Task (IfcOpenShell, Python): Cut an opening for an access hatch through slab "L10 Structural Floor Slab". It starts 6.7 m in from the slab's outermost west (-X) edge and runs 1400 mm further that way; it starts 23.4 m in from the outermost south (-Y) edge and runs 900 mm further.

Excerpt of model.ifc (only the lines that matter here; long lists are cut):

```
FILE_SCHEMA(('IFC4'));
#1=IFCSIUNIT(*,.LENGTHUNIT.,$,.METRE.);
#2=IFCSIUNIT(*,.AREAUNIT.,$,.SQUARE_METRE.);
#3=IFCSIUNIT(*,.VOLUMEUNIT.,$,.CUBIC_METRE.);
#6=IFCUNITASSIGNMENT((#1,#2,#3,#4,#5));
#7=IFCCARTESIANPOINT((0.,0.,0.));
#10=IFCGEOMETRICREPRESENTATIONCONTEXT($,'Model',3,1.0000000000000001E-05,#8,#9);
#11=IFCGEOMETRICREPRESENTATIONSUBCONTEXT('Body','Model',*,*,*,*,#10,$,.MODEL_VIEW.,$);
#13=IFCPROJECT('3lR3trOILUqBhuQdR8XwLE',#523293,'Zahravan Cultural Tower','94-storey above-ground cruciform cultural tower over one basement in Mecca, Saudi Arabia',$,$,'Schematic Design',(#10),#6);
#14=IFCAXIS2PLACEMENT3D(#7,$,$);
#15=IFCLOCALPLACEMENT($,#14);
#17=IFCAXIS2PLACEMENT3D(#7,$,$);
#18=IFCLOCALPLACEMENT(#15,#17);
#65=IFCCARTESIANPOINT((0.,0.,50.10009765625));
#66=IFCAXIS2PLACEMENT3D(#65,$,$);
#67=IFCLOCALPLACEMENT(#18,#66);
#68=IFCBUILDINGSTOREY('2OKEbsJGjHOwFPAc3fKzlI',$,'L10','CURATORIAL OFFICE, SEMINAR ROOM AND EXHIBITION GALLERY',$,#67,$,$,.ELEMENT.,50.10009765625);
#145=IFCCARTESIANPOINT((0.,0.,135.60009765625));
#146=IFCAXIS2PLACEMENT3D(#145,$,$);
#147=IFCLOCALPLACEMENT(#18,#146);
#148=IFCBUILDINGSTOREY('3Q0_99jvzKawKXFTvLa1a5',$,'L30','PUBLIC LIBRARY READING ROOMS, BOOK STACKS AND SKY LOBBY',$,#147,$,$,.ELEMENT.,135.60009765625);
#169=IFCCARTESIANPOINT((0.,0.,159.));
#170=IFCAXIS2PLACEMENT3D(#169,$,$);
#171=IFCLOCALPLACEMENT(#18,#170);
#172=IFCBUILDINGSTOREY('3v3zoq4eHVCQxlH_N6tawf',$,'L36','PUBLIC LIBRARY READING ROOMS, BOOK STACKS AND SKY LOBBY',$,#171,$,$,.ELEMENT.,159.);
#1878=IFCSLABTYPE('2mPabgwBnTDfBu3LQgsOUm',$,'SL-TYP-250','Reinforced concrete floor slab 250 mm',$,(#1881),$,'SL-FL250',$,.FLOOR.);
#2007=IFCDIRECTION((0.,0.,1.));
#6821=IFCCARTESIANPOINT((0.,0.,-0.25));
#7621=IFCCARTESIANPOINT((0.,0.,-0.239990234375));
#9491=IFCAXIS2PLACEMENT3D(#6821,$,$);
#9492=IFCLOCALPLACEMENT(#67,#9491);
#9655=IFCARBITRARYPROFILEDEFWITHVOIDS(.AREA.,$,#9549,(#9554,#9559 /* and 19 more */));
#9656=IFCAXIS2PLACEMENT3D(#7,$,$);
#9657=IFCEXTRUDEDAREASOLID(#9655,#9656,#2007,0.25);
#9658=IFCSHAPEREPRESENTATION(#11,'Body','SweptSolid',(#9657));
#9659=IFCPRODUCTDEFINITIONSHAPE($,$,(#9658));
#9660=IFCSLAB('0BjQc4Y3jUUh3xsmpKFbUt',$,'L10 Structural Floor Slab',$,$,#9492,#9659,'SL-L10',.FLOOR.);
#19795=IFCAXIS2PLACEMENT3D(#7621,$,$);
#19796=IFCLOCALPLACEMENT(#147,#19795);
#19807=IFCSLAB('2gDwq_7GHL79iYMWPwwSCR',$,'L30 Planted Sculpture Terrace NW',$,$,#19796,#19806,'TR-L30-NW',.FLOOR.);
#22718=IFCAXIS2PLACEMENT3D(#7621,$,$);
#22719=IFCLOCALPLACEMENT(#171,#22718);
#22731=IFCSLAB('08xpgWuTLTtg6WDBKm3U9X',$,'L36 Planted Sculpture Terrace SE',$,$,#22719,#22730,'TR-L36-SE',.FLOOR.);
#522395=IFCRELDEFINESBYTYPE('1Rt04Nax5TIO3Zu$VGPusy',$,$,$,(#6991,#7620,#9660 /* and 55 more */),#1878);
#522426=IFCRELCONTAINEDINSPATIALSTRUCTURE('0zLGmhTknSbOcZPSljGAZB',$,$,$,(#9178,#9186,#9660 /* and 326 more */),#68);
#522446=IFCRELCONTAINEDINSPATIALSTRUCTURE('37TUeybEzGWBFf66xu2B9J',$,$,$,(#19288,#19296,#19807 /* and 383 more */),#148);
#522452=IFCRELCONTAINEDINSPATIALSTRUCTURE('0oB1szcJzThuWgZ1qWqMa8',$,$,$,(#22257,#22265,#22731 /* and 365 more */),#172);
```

```python
import numpy as np
import ifcopenshell
import ifcopenshell.api.feature
import ifcopenshell.api.geometry
import ifcopenshell.api.root
import ifcopenshell.geom
import ifcopenshell.util.placement
import ifcopenshell.util.representation
import ifcopenshell.util.shape
import ifcopenshell.util.unit

model = ifcopenshell.open("model.ifc")
unit_scale = ifcopenshell.util.unit.calculate_unit_scale(model)
settings = ifcopenshell.geom.settings()


def volume(element):
    """Net volume in cubic metres, openings subtracted."""
    shape = ifcopenshell.geom.create_shape(settings, element)
    return ifcopenshell.util.shape.get_volume(shape.geometry)


slab = model.by_guid("0BjQc4Y3jUUh3xsmpKFbUt")
before = volume(slab)

# Extent in the slab's own axes, in metres. The edges named are its -X and -Y sides.
slab_shape = ifcopenshell.geom.create_shape(settings, slab)
vertices = ifcopenshell.util.shape.get_vertices(slab_shape.geometry)
x_min, y_min, bottom = vertices.min(axis=0)
top = vertices[:, 2].max()

opening = ifcopenshell.api.root.create_entity(model, ifc_class="IfcOpeningElement", name="Access hatch opening", predefined_type="OPENING")
context = ifcopenshell.util.representation.get_context(model, "Model", "Body", "MODEL_VIEW")
width, depth = 1.4, 0.9
outline = [(0.0, 0.0), (width, 0.0), (width, depth), (0.0, depth), (0.0, 0.0)]
# Overshoot both faces by 50 mm so the cut is clean.
shape = ifcopenshell.api.geometry.add_slab_representation(
    model, context=context, depth=top - bottom + 0.1, polyline=outline
)
ifcopenshell.api.geometry.assign_representation(model, product=opening, representation=shape)

matrix = ifcopenshell.util.placement.get_local_placement(slab.ObjectPlacement)
matrix[:, 3] = matrix @ np.append(np.array([x_min + 6.7, y_min + 23.4, bottom - 0.05]) / unit_scale, 1.0)
ifcopenshell.api.geometry.edit_object_placement(model, product=opening, matrix=matrix, is_si=False)
ifcopenshell.api.feature.add_feature(model, feature=opening, element=slab)

after = volume(slab)

print(f"slab volume {before:.3f} -> {after:.3f} m3")

model.write("model_edited.ifc")
```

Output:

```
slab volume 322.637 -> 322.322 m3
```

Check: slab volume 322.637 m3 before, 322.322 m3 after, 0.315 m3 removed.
